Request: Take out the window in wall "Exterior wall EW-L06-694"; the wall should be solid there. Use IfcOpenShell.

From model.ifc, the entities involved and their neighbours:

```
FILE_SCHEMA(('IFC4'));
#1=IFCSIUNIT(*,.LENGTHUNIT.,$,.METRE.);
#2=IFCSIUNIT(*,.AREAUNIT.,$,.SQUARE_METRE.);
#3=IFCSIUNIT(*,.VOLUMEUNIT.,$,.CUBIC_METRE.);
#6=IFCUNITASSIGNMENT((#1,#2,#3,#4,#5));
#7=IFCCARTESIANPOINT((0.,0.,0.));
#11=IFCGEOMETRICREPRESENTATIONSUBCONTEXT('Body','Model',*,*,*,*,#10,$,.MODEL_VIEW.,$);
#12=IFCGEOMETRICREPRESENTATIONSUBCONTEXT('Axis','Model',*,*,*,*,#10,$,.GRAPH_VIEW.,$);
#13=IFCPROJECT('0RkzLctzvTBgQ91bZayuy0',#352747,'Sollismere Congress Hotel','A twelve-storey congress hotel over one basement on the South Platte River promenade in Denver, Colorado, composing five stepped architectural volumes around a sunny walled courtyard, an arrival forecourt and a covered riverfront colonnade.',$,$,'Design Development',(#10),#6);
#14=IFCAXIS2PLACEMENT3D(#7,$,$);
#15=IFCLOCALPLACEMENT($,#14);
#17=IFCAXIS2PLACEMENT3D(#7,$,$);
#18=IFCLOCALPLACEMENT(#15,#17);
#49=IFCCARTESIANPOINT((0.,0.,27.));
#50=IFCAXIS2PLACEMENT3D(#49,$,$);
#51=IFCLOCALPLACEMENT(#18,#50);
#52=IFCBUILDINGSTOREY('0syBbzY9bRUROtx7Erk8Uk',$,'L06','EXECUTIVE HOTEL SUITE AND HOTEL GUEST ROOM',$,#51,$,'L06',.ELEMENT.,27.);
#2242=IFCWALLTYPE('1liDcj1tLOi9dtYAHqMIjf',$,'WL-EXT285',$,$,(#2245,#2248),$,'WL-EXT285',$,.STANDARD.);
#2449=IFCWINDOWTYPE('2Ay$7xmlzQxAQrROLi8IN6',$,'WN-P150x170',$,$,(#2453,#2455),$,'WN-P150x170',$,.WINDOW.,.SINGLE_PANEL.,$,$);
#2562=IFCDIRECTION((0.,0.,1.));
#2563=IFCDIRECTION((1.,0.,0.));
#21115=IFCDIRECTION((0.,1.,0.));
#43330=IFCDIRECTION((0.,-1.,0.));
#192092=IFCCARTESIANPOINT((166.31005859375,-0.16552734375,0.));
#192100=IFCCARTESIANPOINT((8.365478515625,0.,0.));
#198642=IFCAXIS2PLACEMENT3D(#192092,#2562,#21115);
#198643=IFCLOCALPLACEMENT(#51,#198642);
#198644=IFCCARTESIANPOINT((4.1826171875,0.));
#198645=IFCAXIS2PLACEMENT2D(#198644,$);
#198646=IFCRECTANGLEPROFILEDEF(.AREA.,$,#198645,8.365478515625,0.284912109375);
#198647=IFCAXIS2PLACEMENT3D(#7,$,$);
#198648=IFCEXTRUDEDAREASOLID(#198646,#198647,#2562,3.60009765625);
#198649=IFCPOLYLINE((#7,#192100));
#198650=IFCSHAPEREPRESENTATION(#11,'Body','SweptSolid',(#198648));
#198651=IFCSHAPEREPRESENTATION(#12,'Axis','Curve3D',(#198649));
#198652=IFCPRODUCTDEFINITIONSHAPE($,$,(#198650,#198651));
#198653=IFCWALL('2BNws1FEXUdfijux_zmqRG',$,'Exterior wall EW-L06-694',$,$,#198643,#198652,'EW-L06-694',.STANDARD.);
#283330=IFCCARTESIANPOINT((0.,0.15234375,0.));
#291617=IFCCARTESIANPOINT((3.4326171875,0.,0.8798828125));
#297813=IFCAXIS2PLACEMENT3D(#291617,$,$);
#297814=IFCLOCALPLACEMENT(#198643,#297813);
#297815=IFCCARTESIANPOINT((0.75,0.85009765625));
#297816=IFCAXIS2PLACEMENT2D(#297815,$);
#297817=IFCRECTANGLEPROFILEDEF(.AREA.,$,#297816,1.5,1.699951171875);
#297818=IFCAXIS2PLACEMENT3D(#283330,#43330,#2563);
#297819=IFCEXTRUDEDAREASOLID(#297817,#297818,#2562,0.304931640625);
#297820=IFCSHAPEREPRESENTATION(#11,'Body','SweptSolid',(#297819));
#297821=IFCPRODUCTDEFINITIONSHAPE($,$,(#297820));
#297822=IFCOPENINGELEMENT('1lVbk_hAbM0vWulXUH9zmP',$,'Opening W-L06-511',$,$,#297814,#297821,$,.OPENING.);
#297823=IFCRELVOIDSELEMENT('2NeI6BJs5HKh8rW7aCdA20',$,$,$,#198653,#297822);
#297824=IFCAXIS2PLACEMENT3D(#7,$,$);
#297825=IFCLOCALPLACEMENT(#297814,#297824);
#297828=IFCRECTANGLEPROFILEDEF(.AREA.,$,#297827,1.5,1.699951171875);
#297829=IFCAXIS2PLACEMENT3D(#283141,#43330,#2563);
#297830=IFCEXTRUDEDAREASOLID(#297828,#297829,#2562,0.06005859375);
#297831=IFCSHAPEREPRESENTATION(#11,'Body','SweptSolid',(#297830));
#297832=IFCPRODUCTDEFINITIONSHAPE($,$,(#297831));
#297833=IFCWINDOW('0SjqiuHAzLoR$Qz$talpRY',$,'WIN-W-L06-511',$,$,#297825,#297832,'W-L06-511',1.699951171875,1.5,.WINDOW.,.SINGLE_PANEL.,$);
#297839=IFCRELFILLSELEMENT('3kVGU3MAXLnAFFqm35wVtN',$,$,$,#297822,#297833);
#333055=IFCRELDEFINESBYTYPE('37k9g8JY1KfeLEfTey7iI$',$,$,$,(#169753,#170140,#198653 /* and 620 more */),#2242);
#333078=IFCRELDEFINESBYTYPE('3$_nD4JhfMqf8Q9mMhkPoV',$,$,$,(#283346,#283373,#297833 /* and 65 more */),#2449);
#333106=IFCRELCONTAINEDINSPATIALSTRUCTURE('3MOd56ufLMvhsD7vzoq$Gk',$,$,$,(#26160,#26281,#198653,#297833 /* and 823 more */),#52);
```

```python
import ifcopenshell
import ifcopenshell.api.feature
import ifcopenshell.api.root
import ifcopenshell.geom
import ifcopenshell.util.shape

model = ifcopenshell.open("model.ifc")
settings = ifcopenshell.geom.settings()


def volume(element):
    """Net volume in cubic metres, openings subtracted."""
    shape = ifcopenshell.geom.create_shape(settings, element)
    return ifcopenshell.util.shape.get_volume(shape.geometry)


window = model.by_id(297833)
opening = window.FillsVoids[0].RelatingOpeningElement
wall = opening.VoidsElements[0].RelatingBuildingElement
before = volume(wall)

ifcopenshell.api.root.remove_product(model, product=window)
ifcopenshell.api.feature.remove_feature(model, feature=opening)

after = volume(wall)

print(f"wall volume {before:.3f} -> {after:.3f} m3")

model.write("model-out.ifc")
```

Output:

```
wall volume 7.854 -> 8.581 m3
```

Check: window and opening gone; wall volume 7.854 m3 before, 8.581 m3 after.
